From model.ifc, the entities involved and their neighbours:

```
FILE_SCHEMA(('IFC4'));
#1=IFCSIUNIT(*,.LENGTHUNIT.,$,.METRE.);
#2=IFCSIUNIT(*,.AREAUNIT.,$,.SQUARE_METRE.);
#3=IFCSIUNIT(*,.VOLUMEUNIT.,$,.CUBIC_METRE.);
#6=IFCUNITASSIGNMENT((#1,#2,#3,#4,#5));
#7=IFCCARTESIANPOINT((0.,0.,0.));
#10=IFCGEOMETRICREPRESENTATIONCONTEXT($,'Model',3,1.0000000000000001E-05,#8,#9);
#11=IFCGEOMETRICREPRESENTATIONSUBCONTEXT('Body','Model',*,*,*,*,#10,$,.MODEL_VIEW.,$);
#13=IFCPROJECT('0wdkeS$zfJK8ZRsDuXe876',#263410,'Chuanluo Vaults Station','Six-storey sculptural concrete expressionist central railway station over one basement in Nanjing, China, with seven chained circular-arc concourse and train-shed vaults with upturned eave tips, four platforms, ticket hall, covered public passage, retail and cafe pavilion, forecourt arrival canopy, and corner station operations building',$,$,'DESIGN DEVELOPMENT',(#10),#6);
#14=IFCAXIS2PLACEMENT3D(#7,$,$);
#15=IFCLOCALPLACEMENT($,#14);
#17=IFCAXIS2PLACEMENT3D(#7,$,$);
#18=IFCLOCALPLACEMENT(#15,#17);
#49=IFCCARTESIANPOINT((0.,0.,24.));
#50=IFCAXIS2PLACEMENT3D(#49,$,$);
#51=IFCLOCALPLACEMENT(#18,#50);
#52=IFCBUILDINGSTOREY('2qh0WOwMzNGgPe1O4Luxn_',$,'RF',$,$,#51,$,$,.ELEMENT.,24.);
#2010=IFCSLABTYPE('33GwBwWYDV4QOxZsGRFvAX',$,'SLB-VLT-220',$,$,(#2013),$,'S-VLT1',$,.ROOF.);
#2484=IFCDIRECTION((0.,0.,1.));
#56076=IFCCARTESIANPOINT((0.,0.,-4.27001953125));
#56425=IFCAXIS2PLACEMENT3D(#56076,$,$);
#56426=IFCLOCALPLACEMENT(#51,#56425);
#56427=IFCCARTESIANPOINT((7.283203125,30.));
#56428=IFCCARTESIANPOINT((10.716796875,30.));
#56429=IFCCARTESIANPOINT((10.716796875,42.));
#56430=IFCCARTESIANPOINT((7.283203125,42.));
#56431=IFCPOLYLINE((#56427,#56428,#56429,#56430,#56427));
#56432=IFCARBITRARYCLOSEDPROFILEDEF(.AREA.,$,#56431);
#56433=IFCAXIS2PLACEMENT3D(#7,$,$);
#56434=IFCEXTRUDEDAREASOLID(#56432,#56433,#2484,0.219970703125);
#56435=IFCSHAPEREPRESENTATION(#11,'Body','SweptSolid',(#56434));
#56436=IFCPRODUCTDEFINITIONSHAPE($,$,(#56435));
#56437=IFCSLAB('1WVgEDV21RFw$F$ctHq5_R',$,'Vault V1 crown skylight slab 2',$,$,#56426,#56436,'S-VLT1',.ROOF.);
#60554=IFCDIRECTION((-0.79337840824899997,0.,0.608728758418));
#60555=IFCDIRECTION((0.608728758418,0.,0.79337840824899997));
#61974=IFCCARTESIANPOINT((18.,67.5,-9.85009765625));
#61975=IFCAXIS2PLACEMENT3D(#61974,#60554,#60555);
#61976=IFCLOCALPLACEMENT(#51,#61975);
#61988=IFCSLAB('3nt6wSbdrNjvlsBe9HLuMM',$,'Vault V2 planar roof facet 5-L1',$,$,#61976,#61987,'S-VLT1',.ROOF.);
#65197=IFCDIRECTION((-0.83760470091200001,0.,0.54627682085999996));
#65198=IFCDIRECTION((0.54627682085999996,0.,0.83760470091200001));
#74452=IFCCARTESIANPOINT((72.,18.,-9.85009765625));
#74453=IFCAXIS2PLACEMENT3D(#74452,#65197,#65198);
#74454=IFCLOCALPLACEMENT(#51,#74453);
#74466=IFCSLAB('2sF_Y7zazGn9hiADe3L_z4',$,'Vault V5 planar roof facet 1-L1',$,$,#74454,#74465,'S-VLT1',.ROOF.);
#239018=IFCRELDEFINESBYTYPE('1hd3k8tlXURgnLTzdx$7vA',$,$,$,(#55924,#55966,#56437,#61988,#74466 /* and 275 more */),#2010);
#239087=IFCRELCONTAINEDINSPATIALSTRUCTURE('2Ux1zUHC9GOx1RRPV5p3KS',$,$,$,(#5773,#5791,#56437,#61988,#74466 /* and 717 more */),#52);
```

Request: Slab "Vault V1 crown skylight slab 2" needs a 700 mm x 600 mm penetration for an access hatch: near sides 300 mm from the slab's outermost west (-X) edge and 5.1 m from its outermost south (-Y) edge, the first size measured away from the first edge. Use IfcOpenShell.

```python
import numpy as np
import ifcopenshell
import ifcopenshell.api.feature
import ifcopenshell.api.geometry
import ifcopenshell.api.root
import ifcopenshell.geom
import ifcopenshell.util.placement
import ifcopenshell.util.representation
import ifcopenshell.util.shape
import ifcopenshell.util.unit

model = ifcopenshell.open("model.ifc")
unit_scale = ifcopenshell.util.unit.calculate_unit_scale(model)
settings = ifcopenshell.geom.settings()


def volume(element):
    """Net volume in cubic metres, openings subtracted."""
    shape = ifcopenshell.geom.create_shape(settings, element)
    return ifcopenshell.util.shape.get_volume(shape.geometry)


slab = model.by_id(56437)
before = volume(slab)

# Extent in the slab's own axes, in metres. The edges named are its -X and -Y sides.
slab_shape = ifcopenshell.geom.create_shape(settings, slab)
vertices = ifcopenshell.util.shape.get_vertices(slab_shape.geometry)
x_min, y_min, bottom = vertices.min(axis=0)
top = vertices[:, 2].max()

opening = ifcopenshell.api.root.create_entity(model, ifc_class="IfcOpeningElement", name="Access hatch opening", predefined_type="OPENING")
context = ifcopenshell.util.representation.get_context(model, "Model", "Body", "MODEL_VIEW")
width, depth = 0.7, 0.6
outline = [(0.0, 0.0), (width, 0.0), (width, depth), (0.0, depth), (0.0, 0.0)]
# Overshoot both faces by 50 mm so the cut is clean.
shape = ifcopenshell.api.geometry.add_slab_representation(
    model, context=context, depth=top - bottom + 0.1, polyline=outline
)
ifcopenshell.api.geometry.assign_representation(model, product=opening, representation=shape)

matrix = ifcopenshell.util.placement.get_local_placement(slab.ObjectPlacement)
matrix[:, 3] = matrix @ np.append(np.array([x_min + 0.3, y_min + 5.1, bottom - 0.05]) / unit_scale, 1.0)
ifcopenshell.api.geometry.edit_object_placement(model, product=opening, matrix=matrix, is_si=False)
ifcopenshell.api.feature.add_feature(model, feature=opening, element=slab)

after = volume(slab)

print(f"slab volume {before:.3f} -> {after:.3f} m3")

model.write("model-out.ifc")
```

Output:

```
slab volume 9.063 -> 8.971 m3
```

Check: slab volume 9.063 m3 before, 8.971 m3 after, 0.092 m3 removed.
